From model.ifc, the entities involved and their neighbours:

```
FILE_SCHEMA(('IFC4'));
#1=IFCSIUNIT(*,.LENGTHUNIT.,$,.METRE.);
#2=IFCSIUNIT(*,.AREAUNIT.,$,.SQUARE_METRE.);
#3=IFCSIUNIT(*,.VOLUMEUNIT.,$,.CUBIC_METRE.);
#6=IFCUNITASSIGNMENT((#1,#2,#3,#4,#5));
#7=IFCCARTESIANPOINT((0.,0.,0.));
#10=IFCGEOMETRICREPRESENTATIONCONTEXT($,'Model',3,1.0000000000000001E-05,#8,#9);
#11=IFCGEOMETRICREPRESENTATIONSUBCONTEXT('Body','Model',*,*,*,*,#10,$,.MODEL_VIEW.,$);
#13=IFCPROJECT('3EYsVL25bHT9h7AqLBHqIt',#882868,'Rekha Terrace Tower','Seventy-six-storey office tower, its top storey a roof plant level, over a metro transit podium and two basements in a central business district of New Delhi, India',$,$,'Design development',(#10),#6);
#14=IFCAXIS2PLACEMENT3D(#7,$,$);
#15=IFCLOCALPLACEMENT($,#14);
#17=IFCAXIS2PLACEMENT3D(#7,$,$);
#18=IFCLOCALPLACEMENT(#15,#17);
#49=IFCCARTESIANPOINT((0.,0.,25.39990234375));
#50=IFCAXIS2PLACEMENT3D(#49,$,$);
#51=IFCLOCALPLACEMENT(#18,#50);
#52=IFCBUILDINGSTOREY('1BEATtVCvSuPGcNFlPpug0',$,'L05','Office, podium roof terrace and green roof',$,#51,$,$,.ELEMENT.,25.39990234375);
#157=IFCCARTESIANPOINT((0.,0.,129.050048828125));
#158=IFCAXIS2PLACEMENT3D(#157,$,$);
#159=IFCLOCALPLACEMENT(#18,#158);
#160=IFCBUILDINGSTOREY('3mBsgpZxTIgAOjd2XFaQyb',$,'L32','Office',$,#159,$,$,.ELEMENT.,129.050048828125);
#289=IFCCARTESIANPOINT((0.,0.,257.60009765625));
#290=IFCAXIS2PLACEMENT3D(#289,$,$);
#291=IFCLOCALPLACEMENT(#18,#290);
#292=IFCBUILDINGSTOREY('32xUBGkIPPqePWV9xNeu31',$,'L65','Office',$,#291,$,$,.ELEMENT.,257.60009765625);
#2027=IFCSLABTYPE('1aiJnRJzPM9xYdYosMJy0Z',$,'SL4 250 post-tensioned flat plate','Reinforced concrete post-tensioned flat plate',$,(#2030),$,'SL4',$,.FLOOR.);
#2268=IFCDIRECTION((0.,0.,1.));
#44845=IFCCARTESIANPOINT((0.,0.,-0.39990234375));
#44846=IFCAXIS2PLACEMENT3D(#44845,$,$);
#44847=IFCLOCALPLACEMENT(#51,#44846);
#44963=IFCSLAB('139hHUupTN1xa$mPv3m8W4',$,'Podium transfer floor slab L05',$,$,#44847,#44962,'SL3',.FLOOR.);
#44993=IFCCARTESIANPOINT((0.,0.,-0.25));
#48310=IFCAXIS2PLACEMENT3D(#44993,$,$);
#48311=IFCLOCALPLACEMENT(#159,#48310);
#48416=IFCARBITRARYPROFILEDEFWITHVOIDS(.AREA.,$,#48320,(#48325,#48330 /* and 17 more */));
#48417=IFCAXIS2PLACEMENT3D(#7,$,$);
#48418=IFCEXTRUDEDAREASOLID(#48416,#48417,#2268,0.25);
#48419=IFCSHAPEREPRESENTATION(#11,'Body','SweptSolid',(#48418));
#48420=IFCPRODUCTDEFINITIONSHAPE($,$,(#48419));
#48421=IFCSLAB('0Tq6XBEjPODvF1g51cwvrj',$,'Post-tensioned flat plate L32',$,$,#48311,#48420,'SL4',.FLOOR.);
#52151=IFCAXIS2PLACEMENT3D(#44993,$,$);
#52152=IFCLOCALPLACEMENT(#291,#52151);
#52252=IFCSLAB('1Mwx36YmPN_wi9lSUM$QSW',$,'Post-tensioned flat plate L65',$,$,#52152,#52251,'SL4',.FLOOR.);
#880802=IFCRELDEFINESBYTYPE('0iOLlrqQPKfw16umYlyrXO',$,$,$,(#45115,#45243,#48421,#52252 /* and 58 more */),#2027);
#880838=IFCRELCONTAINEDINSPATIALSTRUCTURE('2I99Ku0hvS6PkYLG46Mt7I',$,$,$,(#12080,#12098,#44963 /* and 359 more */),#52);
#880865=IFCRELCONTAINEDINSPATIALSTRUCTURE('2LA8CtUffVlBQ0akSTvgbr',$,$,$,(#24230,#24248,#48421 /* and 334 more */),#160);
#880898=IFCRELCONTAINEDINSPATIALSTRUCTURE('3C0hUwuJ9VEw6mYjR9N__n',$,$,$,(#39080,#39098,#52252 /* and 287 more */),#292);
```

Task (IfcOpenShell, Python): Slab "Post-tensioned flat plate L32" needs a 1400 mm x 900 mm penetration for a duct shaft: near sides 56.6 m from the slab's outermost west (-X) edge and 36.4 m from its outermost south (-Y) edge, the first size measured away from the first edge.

```python
import numpy as np
import ifcopenshell
import ifcopenshell.api.feature
import ifcopenshell.api.geometry
import ifcopenshell.api.root
import ifcopenshell.geom
import ifcopenshell.util.placement
import ifcopenshell.util.representation
import ifcopenshell.util.shape
import ifcopenshell.util.unit

model = ifcopenshell.open("model.ifc")
unit_scale = ifcopenshell.util.unit.calculate_unit_scale(model)
settings = ifcopenshell.geom.settings()


def volume(element):
    """Net volume in cubic metres, openings subtracted."""
    shape = ifcopenshell.geom.create_shape(settings, element)
    return ifcopenshell.util.shape.get_volume(shape.geometry)


slab = model.by_guid("0Tq6XBEjPODvF1g51cwvrj")
before = volume(slab)

# Extent in the slab's own axes, in metres. The edges named are its -X and -Y sides.
slab_shape = ifcopenshell.geom.create_shape(settings, slab)
vertices = ifcopenshell.util.shape.get_vertices(slab_shape.geometry)
x_min, y_min, bottom = vertices.min(axis=0)
top = vertices[:, 2].max()

opening = ifcopenshell.api.root.create_entity(model, ifc_class="IfcOpeningElement", name="Duct shaft opening", predefined_type="OPENING")
context = ifcopenshell.util.representation.get_context(model, "Model", "Body", "MODEL_VIEW")
width, depth = 1.4, 0.9
outline = [(0.0, 0.0), (width, 0.0), (width, depth), (0.0, depth), (0.0, 0.0)]
# Overshoot both faces by 50 mm so the cut is clean.
shape = ifcopenshell.api.geometry.add_slab_representation(
    model, context=context, depth=top - bottom + 0.1, polyline=outline
)
ifcopenshell.api.geometry.assign_representation(model, product=opening, representation=shape)

matrix = ifcopenshell.util.placement.get_local_placement(slab.ObjectPlacement)
matrix[:, 3] = matrix @ np.append(np.array([x_min + 56.6, y_min + 36.4, bottom - 0.05]) / unit_scale, 1.0)
ifcopenshell.api.geometry.edit_object_placement(model, product=opening, matrix=matrix, is_si=False)
ifcopenshell.api.feature.add_feature(model, feature=opening, element=slab)

after = volume(slab)

print(f"slab volume {before:.3f} -> {after:.3f} m3")

model.write("model-out.ifc")
```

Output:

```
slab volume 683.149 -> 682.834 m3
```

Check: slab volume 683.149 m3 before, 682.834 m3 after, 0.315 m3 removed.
